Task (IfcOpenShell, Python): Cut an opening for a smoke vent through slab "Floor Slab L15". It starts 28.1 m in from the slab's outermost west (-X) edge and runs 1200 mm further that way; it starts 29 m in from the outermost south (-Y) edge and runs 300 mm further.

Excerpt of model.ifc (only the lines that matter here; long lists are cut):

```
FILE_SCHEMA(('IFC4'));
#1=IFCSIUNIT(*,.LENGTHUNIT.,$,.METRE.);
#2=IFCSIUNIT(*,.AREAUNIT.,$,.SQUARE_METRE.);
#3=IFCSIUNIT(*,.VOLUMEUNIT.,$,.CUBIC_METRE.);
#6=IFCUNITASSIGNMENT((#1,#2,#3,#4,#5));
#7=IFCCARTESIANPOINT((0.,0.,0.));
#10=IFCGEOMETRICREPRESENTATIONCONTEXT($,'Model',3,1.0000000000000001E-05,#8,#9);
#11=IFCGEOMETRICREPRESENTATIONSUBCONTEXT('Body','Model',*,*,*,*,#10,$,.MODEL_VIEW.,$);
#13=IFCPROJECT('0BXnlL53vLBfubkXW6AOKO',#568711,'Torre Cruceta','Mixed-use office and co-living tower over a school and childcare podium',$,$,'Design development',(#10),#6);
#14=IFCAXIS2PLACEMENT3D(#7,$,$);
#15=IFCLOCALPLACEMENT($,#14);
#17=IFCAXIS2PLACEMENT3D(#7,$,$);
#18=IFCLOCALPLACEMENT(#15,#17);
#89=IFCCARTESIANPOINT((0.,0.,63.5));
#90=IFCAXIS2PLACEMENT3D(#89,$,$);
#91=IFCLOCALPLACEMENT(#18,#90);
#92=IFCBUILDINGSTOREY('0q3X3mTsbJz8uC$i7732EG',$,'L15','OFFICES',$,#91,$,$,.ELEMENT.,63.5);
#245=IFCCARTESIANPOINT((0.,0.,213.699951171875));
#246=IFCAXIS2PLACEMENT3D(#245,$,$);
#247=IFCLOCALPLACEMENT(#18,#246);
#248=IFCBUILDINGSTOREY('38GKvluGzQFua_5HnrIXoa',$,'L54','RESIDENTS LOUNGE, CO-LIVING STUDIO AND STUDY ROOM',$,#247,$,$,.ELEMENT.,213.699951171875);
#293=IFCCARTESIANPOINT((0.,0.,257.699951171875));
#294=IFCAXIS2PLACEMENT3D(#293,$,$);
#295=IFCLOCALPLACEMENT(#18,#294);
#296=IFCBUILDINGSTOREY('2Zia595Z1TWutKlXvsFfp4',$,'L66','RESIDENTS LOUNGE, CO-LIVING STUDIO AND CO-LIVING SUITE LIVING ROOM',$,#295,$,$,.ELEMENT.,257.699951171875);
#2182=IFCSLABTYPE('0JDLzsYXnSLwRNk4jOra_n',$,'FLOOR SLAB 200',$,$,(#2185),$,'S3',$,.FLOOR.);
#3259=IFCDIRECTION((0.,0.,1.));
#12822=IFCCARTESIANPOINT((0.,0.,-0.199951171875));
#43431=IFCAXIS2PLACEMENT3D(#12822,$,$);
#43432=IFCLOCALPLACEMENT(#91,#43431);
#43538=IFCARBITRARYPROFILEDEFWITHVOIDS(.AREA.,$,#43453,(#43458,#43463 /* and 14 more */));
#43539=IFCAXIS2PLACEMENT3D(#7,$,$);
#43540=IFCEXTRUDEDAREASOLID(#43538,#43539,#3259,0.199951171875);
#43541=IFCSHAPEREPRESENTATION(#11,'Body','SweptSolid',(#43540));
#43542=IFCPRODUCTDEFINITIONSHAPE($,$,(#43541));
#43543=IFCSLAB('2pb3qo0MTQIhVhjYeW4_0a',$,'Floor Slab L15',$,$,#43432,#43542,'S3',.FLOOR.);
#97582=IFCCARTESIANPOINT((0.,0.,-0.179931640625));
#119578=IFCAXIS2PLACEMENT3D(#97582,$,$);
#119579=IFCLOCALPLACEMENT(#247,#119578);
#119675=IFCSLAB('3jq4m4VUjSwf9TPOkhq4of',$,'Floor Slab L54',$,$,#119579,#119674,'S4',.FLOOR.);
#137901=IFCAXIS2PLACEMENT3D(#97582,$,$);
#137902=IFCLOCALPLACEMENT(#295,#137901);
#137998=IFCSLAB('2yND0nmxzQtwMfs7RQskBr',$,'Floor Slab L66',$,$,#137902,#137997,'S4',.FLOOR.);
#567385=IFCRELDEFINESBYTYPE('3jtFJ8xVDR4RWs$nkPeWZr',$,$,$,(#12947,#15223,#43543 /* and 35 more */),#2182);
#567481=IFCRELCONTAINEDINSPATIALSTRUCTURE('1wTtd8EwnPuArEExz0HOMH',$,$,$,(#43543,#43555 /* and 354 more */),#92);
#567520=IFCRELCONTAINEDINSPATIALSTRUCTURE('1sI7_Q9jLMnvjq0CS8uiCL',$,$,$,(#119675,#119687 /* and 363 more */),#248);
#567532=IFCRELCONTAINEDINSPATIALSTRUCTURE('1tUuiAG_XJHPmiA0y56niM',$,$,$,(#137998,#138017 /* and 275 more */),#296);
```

```python
import numpy as np
import ifcopenshell
import ifcopenshell.api.feature
import ifcopenshell.api.geometry
import ifcopenshell.api.root
import ifcopenshell.geom
import ifcopenshell.util.placement
import ifcopenshell.util.representation
import ifcopenshell.util.shape
import ifcopenshell.util.unit

model = ifcopenshell.open("model.ifc")
unit_scale = ifcopenshell.util.unit.calculate_unit_scale(model)
settings = ifcopenshell.geom.settings()


def volume(element):
    """Net volume in cubic metres, openings subtracted."""
    shape = ifcopenshell.geom.create_shape(settings, element)
    return ifcopenshell.util.shape.get_volume(shape.geometry)


slab = model.by_guid("2pb3qo0MTQIhVhjYeW4_0a")
before = volume(slab)

# Extent in the slab's own axes, in metres. The edges named are its -X and -Y sides.
slab_shape = ifcopenshell.geom.create_shape(settings, slab)
vertices = ifcopenshell.util.shape.get_vertices(slab_shape.geometry)
x_min, y_min, bottom = vertices.min(axis=0)
top = vertices[:, 2].max()

opening = ifcopenshell.api.root.create_entity(model, ifc_class="IfcOpeningElement", name="Smoke vent opening", predefined_type="OPENING")
context = ifcopenshell.util.representation.get_context(model, "Model", "Body", "MODEL_VIEW")
width, depth = 1.2, 0.3
outline = [(0.0, 0.0), (width, 0.0), (width, depth), (0.0, depth), (0.0, 0.0)]
# Overshoot both faces by 50 mm so the cut is clean.
shape = ifcopenshell.api.geometry.add_slab_representation(
    model, context=context, depth=top - bottom + 0.1, polyline=outline
)
ifcopenshell.api.geometry.assign_representation(model, product=opening, representation=shape)

matrix = ifcopenshell.util.placement.get_local_placement(slab.ObjectPlacement)
matrix[:, 3] = matrix @ np.append(np.array([x_min + 28.1, y_min + 29, bottom - 0.05]) / unit_scale, 1.0)
ifcopenshell.api.geometry.edit_object_placement(model, product=opening, matrix=matrix, is_si=False)
ifcopenshell.api.feature.add_feature(model, feature=opening, element=slab)

after = volume(slab)

print(f"slab volume {before:.3f} -> {after:.3f} m3")

model.write("model_edited.ifc")
```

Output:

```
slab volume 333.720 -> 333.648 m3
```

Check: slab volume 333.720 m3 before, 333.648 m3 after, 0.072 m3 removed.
